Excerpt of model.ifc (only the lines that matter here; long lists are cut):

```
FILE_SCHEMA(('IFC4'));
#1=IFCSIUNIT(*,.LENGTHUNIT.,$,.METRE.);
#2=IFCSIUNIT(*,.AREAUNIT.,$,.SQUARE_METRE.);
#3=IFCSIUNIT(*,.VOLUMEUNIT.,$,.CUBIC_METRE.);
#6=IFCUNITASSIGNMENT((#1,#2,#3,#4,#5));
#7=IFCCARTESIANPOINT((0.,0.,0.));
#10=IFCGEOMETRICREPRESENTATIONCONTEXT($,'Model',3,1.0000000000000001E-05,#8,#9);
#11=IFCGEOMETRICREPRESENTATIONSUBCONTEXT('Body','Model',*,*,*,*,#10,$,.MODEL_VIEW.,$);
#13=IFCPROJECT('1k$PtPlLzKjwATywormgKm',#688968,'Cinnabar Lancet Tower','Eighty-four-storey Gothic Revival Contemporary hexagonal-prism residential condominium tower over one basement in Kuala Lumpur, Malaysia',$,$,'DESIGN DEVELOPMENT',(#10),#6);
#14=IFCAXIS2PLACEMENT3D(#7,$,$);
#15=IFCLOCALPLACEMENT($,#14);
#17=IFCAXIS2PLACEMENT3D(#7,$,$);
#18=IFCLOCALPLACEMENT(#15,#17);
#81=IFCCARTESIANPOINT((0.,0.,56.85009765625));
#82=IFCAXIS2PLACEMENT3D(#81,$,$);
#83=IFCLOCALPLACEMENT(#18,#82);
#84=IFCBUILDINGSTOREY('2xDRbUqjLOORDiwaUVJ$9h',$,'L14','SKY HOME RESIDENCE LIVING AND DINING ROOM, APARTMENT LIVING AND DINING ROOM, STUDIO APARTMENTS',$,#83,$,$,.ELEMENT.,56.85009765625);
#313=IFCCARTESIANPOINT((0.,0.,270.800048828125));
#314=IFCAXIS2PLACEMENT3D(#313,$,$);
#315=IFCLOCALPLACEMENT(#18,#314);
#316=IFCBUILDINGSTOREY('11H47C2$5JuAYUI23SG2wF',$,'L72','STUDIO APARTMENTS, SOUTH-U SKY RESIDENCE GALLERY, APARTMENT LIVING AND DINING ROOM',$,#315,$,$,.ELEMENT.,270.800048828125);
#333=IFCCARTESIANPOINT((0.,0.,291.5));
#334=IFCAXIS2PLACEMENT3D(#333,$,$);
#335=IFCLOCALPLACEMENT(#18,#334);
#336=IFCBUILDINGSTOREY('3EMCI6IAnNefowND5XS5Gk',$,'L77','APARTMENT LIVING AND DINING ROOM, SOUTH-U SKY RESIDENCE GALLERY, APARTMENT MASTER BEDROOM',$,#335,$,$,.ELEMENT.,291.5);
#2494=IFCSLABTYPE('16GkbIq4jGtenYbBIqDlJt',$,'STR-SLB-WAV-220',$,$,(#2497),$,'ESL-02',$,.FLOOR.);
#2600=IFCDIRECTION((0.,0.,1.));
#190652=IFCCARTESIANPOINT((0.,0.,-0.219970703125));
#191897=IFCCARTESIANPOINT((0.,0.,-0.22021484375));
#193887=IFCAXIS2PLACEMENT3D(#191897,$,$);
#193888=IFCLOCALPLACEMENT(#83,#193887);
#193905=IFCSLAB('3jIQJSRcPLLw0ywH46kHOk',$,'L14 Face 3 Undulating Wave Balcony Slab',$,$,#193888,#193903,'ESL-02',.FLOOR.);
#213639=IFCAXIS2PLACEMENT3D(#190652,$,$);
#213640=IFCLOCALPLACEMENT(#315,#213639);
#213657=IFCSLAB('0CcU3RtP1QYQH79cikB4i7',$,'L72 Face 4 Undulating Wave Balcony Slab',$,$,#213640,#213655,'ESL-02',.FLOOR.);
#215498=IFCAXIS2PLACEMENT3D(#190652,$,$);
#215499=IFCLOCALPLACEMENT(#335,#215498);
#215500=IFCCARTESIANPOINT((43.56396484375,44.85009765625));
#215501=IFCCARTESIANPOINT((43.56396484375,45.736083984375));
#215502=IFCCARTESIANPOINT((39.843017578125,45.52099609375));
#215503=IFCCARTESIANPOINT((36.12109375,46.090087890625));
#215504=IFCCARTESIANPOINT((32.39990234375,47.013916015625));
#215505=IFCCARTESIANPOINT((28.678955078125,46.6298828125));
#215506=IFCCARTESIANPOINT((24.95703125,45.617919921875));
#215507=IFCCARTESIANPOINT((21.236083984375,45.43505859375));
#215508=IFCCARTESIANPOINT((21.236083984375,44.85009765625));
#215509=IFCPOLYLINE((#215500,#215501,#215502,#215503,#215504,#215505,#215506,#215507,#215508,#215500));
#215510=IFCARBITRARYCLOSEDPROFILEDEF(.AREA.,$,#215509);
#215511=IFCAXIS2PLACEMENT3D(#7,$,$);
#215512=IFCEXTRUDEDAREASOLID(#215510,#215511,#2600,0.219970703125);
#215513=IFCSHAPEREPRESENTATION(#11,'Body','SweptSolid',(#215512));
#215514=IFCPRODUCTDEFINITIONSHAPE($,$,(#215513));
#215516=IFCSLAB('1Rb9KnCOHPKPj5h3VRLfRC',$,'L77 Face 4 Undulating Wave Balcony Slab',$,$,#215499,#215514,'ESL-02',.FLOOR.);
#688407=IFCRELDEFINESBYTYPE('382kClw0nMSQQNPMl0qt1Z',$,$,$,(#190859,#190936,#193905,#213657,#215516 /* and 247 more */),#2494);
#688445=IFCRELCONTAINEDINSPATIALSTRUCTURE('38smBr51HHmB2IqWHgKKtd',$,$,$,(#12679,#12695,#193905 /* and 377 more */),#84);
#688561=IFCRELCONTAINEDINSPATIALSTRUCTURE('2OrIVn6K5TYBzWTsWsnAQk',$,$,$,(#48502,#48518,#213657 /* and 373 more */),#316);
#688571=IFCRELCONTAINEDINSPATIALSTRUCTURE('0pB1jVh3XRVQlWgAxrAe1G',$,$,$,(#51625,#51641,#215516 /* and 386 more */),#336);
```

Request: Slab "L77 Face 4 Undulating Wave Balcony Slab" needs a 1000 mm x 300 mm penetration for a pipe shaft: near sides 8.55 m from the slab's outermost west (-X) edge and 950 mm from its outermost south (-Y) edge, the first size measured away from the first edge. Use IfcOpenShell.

```python
import numpy as np
import ifcopenshell
import ifcopenshell.api.feature
import ifcopenshell.api.geometry
import ifcopenshell.api.root
import ifcopenshell.geom
import ifcopenshell.util.placement
import ifcopenshell.util.representation
import ifcopenshell.util.shape
import ifcopenshell.util.unit

model = ifcopenshell.open("model.ifc")
unit_scale = ifcopenshell.util.unit.calculate_unit_scale(model)
settings = ifcopenshell.geom.settings()


def volume(element):
    """Net volume in cubic metres, openings subtracted."""
    shape = ifcopenshell.geom.create_shape(settings, element)
    return ifcopenshell.util.shape.get_volume(shape.geometry)


slab = model.by_id(215516)
before = volume(slab)

# Extent in the slab's own axes, in metres. The edges named are its -X and -Y sides.
slab_shape = ifcopenshell.geom.create_shape(settings, slab)
vertices = ifcopenshell.util.shape.get_vertices(slab_shape.geometry)
x_min, y_min, bottom = vertices.min(axis=0)
top = vertices[:, 2].max()

opening = ifcopenshell.api.root.create_entity(model, ifc_class="IfcOpeningElement", name="Pipe shaft opening", predefined_type="OPENING")
context = ifcopenshell.util.representation.get_context(model, "Model", "Body", "MODEL_VIEW")
width, depth = 1, 0.3
outline = [(0.0, 0.0), (width, 0.0), (width, depth), (0.0, depth), (0.0, 0.0)]
# Overshoot both faces by 50 mm so the cut is clean.
shape = ifcopenshell.api.geometry.add_slab_representation(
    model, context=context, depth=top - bottom + 0.1, polyline=outline
)
ifcopenshell.api.geometry.assign_representation(model, product=opening, representation=shape)

matrix = ifcopenshell.util.placement.get_local_placement(slab.ObjectPlacement)
matrix[:, 3] = matrix @ np.append(np.array([x_min + 8.55, y_min + 0.95, bottom - 0.05]) / unit_scale, 1.0)
ifcopenshell.api.geometry.edit_object_placement(model, product=opening, matrix=matrix, is_si=False)
ifcopenshell.api.feature.add_feature(model, feature=opening, element=slab)

after = volume(slab)

print(f"slab volume {before:.3f} -> {after:.3f} m3")

model.write("model_v2.ifc")
```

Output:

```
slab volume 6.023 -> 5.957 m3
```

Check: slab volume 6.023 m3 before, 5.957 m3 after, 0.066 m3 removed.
